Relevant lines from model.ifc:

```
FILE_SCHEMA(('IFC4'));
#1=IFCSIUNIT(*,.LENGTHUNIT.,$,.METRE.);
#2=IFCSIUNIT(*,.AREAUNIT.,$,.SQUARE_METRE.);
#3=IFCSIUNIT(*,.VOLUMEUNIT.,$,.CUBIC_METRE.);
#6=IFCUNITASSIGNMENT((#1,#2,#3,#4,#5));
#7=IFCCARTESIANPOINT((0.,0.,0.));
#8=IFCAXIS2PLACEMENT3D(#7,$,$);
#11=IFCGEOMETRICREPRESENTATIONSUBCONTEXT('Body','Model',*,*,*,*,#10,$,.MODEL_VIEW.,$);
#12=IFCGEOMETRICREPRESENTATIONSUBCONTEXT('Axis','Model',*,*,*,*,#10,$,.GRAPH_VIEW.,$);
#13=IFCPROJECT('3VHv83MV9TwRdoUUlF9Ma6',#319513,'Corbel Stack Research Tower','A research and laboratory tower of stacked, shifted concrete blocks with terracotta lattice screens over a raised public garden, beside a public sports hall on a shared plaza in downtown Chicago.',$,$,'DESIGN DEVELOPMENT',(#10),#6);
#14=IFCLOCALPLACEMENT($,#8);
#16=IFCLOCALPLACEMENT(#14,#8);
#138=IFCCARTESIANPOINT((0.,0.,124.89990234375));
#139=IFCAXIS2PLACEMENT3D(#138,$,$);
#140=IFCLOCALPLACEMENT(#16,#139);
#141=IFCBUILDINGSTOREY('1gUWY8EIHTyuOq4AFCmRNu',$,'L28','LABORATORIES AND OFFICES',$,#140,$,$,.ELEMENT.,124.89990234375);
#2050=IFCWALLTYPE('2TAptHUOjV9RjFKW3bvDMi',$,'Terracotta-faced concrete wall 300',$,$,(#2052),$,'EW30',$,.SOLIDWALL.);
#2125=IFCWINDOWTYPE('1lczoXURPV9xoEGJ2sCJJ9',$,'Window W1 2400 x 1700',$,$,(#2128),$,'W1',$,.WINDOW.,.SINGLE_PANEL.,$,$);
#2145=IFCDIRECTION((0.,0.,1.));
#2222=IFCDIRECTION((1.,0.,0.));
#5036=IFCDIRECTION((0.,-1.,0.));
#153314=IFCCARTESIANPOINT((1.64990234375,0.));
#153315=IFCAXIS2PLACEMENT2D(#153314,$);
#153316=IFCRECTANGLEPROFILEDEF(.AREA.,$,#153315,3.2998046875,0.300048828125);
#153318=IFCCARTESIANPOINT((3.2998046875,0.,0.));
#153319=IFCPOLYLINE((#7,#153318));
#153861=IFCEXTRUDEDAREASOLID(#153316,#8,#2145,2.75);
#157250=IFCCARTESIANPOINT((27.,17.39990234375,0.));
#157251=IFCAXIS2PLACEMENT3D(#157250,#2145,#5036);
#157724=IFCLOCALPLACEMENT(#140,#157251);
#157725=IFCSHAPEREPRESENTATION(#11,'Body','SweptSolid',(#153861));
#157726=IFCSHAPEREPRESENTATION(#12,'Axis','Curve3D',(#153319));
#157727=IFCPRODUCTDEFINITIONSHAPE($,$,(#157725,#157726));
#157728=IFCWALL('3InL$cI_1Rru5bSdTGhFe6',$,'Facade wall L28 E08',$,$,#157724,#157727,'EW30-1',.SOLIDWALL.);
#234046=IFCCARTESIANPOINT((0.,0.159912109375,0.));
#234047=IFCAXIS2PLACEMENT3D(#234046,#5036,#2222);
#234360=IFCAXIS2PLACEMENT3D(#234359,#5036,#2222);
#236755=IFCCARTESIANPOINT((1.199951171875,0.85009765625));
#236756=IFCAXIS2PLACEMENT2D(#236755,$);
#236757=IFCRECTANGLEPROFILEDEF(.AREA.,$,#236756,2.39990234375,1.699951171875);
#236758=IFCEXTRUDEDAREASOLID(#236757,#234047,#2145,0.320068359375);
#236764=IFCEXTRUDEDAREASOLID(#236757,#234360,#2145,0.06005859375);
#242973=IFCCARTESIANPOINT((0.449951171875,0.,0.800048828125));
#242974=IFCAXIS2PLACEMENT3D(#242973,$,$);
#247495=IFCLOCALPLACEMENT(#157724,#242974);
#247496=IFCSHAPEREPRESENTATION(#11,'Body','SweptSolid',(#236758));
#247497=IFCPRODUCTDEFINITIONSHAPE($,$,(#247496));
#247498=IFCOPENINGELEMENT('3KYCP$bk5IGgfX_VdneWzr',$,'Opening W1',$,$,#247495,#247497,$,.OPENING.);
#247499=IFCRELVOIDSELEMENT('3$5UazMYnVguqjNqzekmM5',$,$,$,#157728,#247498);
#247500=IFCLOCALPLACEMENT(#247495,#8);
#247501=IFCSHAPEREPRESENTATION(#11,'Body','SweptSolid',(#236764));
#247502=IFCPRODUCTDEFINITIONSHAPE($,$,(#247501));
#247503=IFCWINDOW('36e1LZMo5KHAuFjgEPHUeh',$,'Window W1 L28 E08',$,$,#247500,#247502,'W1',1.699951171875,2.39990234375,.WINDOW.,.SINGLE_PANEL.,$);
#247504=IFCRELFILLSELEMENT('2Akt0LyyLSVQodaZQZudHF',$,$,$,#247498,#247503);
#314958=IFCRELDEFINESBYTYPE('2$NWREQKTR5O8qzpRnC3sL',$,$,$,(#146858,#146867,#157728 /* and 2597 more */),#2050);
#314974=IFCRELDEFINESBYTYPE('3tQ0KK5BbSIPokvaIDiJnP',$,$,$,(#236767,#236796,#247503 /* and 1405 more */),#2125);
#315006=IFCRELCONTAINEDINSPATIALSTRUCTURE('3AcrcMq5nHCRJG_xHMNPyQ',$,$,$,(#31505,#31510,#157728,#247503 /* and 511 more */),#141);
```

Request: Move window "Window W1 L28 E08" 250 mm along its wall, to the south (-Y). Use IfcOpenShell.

```python
import ifcopenshell
import ifcopenshell.api.geometry
import ifcopenshell.util.placement

model = ifcopenshell.open("model.ifc")

window = model.by_id(247503)
opening = window.FillsVoids[0].RelatingOpeningElement
wall = opening.VoidsElements[0].RelatingBuildingElement

wall_matrix = ifcopenshell.util.placement.get_local_placement(wall.ObjectPlacement)
shift = wall_matrix[:3, 0] * 0.25
before = ifcopenshell.util.placement.get_local_placement(window.ObjectPlacement)[:3, 3].copy()

# The window is placed relative to its opening, so it follows when the opening moves.
matrix = ifcopenshell.util.placement.get_local_placement(opening.ObjectPlacement)
matrix[:3, 3] += shift
ifcopenshell.api.geometry.edit_object_placement(
    model, product=opening, matrix=matrix, is_si=False, should_transform_children=True
)

after = ifcopenshell.util.placement.get_local_placement(window.ObjectPlacement)[:3, 3]
print("window moved by", (after - before).round(3) + 0.0)

model.write("model_updated.ifc")
```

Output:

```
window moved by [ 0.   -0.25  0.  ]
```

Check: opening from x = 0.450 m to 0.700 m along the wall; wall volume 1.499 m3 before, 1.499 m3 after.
